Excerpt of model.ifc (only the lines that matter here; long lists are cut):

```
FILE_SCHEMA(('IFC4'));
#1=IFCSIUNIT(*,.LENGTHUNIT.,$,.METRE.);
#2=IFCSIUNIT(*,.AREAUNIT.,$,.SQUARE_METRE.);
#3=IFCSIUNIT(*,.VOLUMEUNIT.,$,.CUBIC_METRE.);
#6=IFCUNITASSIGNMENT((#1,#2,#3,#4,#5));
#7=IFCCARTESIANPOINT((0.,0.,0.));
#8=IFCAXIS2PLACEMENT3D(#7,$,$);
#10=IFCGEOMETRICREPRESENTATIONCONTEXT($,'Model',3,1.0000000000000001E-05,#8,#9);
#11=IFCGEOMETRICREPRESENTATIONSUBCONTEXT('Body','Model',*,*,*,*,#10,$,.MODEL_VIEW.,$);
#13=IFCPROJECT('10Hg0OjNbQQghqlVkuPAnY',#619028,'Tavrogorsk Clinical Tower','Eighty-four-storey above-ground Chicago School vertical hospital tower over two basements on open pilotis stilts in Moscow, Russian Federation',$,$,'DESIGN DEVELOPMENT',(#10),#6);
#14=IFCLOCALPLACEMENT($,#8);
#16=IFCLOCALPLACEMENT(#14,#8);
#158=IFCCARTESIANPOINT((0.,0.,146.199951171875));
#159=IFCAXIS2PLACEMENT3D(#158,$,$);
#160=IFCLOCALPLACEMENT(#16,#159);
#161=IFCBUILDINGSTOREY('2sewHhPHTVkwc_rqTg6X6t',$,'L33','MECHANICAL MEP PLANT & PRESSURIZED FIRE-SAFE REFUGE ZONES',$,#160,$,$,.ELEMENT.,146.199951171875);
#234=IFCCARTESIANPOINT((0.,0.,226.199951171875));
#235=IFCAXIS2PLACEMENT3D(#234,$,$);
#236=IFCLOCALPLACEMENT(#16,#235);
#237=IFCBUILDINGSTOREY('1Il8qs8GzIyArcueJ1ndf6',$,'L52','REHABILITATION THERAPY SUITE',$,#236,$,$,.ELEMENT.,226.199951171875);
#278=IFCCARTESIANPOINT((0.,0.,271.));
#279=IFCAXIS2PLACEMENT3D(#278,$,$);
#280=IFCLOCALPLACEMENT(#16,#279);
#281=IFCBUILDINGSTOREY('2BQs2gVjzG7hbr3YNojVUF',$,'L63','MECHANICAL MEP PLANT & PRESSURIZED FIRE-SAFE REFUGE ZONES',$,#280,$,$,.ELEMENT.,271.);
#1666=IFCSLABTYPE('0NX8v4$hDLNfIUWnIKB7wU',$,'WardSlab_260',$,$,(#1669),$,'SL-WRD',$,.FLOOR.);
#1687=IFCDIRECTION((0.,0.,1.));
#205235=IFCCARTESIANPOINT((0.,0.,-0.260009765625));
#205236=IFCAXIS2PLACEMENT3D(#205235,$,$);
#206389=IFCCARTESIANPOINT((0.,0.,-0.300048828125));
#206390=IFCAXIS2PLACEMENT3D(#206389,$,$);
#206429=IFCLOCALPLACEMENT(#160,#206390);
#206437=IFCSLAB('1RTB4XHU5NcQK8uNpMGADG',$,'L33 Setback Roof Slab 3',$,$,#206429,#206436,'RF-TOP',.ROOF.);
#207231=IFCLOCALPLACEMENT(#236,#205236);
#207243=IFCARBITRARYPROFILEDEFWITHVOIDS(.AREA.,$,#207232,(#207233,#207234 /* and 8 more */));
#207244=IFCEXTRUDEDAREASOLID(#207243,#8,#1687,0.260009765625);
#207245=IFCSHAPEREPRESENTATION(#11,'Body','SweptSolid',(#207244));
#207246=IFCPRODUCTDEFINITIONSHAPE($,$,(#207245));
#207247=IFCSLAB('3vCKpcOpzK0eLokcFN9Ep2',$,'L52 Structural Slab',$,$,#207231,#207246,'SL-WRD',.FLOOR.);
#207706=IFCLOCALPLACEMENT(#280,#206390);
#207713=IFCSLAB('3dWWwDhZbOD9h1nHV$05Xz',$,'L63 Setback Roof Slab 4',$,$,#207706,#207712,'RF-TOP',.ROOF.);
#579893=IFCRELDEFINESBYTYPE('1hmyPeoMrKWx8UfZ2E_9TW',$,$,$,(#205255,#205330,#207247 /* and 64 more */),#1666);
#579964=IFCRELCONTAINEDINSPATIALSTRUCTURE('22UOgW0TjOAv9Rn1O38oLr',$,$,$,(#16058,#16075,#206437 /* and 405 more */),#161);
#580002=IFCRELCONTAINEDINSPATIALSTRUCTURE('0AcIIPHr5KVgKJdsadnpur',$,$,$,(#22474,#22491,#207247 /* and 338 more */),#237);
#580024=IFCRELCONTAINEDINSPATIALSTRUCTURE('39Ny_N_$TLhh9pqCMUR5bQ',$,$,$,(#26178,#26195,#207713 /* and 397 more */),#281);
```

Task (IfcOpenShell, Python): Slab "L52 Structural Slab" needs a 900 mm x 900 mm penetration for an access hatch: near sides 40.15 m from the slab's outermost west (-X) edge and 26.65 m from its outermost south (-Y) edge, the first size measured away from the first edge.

```python
import numpy as np
import ifcopenshell
import ifcopenshell.api.feature
import ifcopenshell.api.geometry
import ifcopenshell.api.root
import ifcopenshell.geom
import ifcopenshell.util.placement
import ifcopenshell.util.representation
import ifcopenshell.util.shape
import ifcopenshell.util.unit

model = ifcopenshell.open("model.ifc")
unit_scale = ifcopenshell.util.unit.calculate_unit_scale(model)
settings = ifcopenshell.geom.settings()


def volume(element):
    """Net volume in cubic metres, openings subtracted."""
    shape = ifcopenshell.geom.create_shape(settings, element)
    return ifcopenshell.util.shape.get_volume(shape.geometry)


slab = model.by_guid("3vCKpcOpzK0eLokcFN9Ep2")
before = volume(slab)

# Extent in the slab's own axes, in metres. The edges named are its -X and -Y sides.
slab_shape = ifcopenshell.geom.create_shape(settings, slab)
vertices = ifcopenshell.util.shape.get_vertices(slab_shape.geometry)
x_min, y_min, bottom = vertices.min(axis=0)
top = vertices[:, 2].max()

opening = ifcopenshell.api.root.create_entity(model, ifc_class="IfcOpeningElement", name="Access hatch opening", predefined_type="OPENING")
context = ifcopenshell.util.representation.get_context(model, "Model", "Body", "MODEL_VIEW")
width, depth = 0.9, 0.9
outline = [(0.0, 0.0), (width, 0.0), (width, depth), (0.0, depth), (0.0, 0.0)]
# Overshoot both faces by 50 mm so the cut is clean.
shape = ifcopenshell.api.geometry.add_slab_representation(
    model, context=context, depth=top - bottom + 0.1, polyline=outline
)
ifcopenshell.api.geometry.assign_representation(model, product=opening, representation=shape)

matrix = ifcopenshell.util.placement.get_local_placement(slab.ObjectPlacement)
matrix[:, 3] = matrix @ np.append(np.array([x_min + 40.15, y_min + 26.65, bottom - 0.05]) / unit_scale, 1.0)
ifcopenshell.api.geometry.edit_object_placement(model, product=opening, matrix=matrix, is_si=False)
ifcopenshell.api.feature.add_feature(model, feature=opening, element=slab)

after = volume(slab)

print(f"slab volume {before:.3f} -> {after:.3f} m3")

model.write("model_updated.ifc")
```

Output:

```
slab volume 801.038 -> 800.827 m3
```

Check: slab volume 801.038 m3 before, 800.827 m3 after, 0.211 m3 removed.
